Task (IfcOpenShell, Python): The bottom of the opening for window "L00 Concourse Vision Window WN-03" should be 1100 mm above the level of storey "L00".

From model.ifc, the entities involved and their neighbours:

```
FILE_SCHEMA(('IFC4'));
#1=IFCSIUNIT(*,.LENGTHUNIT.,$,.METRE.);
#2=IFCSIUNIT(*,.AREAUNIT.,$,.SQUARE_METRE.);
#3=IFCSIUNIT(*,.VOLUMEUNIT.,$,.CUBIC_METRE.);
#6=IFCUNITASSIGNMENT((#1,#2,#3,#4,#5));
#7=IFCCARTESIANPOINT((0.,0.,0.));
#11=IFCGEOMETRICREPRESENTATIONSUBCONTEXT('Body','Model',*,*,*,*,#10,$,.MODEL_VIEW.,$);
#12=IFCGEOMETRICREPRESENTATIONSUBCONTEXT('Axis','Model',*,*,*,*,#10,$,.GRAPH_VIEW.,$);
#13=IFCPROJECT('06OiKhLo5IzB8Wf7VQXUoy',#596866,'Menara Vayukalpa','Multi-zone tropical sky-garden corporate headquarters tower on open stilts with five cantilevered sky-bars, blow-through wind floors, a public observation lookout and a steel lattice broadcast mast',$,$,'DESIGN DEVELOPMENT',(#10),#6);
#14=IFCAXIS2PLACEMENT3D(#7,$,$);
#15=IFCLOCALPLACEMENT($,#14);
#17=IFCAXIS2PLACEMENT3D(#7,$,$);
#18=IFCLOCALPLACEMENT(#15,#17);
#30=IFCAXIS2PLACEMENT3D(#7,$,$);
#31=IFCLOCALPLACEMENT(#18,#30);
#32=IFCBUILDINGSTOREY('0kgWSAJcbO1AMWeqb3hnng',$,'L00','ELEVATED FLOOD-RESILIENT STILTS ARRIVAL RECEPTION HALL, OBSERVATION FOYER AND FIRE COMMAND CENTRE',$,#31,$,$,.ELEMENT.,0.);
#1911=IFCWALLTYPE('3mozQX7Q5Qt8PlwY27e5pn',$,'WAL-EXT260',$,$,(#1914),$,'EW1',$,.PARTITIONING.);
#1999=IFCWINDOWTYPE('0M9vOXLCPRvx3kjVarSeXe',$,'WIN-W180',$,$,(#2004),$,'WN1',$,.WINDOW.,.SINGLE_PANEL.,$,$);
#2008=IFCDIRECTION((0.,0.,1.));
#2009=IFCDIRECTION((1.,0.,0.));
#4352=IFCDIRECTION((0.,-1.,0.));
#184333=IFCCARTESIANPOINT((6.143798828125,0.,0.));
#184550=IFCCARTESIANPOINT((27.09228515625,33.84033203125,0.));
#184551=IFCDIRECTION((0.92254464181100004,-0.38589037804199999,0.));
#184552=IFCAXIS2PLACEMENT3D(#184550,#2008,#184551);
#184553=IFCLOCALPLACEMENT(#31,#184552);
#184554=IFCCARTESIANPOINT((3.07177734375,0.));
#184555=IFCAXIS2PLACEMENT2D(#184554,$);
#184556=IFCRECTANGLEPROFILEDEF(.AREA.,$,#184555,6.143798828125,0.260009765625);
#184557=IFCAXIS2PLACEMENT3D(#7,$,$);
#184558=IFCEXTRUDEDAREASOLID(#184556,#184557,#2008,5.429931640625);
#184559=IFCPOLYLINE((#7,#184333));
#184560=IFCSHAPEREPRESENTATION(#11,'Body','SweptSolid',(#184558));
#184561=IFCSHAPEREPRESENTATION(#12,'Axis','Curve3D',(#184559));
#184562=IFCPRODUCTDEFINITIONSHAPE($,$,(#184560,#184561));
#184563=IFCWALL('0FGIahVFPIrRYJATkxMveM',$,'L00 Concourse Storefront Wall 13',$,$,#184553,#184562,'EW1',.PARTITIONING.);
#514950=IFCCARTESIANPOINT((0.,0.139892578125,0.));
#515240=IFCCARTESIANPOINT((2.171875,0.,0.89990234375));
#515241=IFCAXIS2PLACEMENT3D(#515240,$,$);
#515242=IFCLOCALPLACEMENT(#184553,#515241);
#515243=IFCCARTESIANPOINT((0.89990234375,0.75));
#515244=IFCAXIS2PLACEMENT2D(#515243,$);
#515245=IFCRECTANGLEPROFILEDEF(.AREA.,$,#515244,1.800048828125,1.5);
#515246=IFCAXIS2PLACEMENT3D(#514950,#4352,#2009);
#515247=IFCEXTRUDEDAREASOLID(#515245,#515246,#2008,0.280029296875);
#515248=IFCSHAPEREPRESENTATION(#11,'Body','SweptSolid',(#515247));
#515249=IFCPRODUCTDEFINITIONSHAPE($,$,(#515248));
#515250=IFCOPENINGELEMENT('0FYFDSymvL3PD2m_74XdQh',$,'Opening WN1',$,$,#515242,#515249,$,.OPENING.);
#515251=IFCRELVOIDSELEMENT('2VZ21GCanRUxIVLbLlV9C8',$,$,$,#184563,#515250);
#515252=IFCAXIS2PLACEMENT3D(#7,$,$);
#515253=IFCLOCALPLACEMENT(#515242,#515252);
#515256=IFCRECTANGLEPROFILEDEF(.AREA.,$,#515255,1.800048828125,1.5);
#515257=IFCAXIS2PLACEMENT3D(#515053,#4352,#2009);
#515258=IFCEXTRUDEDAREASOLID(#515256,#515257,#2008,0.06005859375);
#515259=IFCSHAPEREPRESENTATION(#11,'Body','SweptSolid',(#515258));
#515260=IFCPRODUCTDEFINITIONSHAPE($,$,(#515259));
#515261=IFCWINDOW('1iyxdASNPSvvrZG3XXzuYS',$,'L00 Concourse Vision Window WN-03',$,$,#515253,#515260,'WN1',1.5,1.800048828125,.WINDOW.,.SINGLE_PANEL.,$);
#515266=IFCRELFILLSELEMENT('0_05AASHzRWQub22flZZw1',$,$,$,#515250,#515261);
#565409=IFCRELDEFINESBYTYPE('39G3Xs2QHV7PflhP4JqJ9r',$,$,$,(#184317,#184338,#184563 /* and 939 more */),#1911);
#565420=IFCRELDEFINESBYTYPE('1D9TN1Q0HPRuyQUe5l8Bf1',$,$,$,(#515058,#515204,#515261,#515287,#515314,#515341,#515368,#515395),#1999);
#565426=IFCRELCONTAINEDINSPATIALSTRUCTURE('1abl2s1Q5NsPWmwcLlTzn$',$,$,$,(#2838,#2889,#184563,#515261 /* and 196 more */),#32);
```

```python
import numpy as np
import ifcopenshell
import ifcopenshell.api.geometry
import ifcopenshell.geom
import ifcopenshell.util.element
import ifcopenshell.util.placement
import ifcopenshell.util.shape
import ifcopenshell.util.unit

model = ifcopenshell.open("model.ifc")
unit_scale = ifcopenshell.util.unit.calculate_unit_scale(model)

window = model.by_id(515261)
opening = window.FillsVoids[0].RelatingOpeningElement
storey = ifcopenshell.util.element.get_container(window, ifc_class="IfcBuildingStorey")
level = ifcopenshell.util.placement.get_local_placement(storey.ObjectPlacement)[2, 3]

# The opening's origin need not be at the sill, so measure its lowest point.
shape = ifcopenshell.geom.create_shape(ifcopenshell.geom.settings(), opening)
bottom = ifcopenshell.util.shape.get_shape_bottom_elevation(shape, shape.geometry) / unit_scale
dz = level + 1.1 / unit_scale - bottom

shift = np.array([0.0, 0.0, dz])
# The window is placed relative to its opening, so it follows when the opening moves.
matrix = ifcopenshell.util.placement.get_local_placement(opening.ObjectPlacement)
matrix[:3, 3] += shift
ifcopenshell.api.geometry.edit_object_placement(
    model, product=opening, matrix=matrix, is_si=False, should_transform_children=True
)

print(f"moved by {dz * unit_scale:+.3f} m")

model.write("model_updated.ifc")
```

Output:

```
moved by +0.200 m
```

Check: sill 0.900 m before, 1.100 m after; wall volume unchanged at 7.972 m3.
